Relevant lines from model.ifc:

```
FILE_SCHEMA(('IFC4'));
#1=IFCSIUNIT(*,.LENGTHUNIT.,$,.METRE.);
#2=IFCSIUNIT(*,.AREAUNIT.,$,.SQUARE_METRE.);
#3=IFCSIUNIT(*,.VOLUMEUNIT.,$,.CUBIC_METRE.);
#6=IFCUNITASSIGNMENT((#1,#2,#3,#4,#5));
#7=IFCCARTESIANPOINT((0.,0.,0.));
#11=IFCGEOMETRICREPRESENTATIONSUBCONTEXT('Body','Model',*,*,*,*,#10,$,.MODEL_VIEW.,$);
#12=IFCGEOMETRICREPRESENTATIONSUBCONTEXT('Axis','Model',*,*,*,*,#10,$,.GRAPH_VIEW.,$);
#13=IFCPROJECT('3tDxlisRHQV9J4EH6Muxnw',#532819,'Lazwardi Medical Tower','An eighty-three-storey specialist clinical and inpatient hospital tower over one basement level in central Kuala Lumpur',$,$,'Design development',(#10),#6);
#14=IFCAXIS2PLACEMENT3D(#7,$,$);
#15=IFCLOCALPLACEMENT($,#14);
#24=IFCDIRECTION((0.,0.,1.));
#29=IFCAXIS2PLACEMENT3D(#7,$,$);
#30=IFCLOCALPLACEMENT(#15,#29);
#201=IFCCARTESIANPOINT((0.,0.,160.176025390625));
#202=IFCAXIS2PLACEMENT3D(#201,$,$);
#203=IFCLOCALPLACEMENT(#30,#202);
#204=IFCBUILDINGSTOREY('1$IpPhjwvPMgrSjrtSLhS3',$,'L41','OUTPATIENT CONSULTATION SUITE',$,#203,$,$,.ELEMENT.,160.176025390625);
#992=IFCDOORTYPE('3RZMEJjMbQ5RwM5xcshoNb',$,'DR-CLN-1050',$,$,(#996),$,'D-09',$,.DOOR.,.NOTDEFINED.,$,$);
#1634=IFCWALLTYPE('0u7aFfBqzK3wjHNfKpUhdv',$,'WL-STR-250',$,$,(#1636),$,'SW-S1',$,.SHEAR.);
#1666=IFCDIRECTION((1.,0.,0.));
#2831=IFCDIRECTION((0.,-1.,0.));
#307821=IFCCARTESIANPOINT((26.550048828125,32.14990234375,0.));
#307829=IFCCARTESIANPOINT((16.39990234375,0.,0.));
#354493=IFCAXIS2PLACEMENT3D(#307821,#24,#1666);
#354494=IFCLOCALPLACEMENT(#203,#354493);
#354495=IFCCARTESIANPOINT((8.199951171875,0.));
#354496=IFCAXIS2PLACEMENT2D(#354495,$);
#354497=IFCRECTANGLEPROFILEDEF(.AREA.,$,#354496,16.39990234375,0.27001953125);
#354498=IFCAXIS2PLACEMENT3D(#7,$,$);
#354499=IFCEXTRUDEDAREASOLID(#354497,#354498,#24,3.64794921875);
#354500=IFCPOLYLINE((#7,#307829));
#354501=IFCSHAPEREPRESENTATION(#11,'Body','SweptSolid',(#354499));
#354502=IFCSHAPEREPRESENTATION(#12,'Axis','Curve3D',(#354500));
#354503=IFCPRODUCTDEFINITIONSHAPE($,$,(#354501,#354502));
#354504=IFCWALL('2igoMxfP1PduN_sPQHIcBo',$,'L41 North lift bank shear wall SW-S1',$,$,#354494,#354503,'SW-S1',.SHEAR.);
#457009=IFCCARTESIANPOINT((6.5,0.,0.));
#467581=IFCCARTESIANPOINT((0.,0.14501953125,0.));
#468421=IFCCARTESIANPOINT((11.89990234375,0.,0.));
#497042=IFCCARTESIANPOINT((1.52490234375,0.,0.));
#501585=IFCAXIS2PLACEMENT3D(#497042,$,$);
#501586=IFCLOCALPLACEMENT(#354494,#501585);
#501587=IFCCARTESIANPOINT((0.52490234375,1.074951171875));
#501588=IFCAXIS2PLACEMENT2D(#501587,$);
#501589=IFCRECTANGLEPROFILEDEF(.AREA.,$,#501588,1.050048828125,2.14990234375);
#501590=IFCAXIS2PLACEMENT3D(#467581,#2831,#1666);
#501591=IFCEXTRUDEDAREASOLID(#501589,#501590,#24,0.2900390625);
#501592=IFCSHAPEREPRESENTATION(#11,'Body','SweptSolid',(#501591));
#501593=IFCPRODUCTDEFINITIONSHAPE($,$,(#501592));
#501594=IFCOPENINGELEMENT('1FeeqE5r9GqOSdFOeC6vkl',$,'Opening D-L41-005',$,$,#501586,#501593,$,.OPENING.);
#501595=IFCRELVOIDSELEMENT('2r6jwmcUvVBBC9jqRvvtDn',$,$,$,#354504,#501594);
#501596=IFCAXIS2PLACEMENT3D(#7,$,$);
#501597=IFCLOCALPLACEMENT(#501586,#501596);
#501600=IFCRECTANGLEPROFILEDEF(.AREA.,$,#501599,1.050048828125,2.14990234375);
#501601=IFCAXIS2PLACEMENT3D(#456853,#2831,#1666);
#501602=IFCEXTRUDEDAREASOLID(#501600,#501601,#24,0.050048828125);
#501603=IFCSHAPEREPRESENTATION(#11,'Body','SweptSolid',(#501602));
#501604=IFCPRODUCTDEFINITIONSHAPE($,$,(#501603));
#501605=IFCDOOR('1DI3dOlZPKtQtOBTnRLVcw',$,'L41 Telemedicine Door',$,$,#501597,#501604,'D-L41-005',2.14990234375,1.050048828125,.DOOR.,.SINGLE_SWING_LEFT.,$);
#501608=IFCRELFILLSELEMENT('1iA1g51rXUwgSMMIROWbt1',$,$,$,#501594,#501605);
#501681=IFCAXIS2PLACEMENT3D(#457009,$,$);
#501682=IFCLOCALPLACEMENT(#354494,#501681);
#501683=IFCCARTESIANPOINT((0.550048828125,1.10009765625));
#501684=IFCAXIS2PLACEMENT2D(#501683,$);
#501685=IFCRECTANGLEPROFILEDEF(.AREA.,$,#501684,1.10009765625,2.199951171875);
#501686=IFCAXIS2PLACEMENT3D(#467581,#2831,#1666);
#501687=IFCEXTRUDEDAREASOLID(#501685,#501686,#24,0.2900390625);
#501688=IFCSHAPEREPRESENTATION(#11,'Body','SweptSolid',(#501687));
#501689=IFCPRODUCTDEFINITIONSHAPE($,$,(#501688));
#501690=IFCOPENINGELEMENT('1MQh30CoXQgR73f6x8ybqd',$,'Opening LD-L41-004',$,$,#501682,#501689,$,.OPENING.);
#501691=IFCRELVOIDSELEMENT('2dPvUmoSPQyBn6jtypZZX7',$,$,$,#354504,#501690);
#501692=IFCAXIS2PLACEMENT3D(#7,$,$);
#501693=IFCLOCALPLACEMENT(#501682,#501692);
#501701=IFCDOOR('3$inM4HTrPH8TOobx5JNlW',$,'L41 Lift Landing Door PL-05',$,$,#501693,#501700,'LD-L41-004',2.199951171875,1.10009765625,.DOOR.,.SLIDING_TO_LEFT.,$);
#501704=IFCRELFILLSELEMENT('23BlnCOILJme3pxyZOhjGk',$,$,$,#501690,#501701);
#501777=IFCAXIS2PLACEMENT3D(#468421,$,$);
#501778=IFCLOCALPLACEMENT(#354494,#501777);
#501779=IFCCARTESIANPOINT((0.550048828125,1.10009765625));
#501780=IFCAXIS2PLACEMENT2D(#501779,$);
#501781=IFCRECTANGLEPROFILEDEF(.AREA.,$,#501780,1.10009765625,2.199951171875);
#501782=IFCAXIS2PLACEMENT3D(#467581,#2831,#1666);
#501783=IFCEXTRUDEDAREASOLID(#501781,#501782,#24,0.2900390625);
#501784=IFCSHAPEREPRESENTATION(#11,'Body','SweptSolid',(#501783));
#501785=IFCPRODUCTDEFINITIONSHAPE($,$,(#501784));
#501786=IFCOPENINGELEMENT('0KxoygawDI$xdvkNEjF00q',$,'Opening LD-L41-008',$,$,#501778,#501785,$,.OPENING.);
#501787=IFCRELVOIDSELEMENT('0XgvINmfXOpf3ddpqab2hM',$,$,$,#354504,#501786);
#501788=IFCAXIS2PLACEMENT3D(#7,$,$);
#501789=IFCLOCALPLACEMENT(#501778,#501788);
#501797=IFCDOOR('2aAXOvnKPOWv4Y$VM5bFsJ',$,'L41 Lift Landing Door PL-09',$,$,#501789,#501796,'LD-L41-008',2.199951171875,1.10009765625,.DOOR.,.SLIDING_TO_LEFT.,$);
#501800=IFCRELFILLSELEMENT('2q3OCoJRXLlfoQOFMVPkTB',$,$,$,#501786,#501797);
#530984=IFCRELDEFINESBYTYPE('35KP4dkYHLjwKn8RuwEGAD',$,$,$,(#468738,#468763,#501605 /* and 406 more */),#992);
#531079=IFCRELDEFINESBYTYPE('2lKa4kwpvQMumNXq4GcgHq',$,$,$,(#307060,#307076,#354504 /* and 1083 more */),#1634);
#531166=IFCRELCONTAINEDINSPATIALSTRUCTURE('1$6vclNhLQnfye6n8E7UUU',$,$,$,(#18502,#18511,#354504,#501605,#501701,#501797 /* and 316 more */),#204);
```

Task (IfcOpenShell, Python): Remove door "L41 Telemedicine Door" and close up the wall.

```python
import ifcopenshell
import ifcopenshell.api.feature
import ifcopenshell.api.root
import ifcopenshell.geom
import ifcopenshell.util.shape

model = ifcopenshell.open("model.ifc")
settings = ifcopenshell.geom.settings()


def volume(element):
    """Net volume in cubic metres, openings subtracted."""
    shape = ifcopenshell.geom.create_shape(settings, element)
    return ifcopenshell.util.shape.get_volume(shape.geometry)


door = model.by_guid("1DI3dOlZPKtQtOBTnRLVcw")
opening = door.FillsVoids[0].RelatingOpeningElement
wall = opening.VoidsElements[0].RelatingBuildingElement
before = volume(wall)

ifcopenshell.api.root.remove_product(model, product=door)
ifcopenshell.api.feature.remove_feature(model, feature=opening)

after = volume(wall)

print(f"wall volume {before:.3f} -> {after:.3f} m3")

model.write("model_edited.ifc")
```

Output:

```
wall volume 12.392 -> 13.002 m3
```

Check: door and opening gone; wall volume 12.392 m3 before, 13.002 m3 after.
